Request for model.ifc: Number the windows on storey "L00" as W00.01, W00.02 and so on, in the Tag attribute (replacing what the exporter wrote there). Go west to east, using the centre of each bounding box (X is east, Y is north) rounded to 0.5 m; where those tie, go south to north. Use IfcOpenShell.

First a look at what the model holds.

```python
import ifcopenshell
import ifcopenshell.util.element
import ifcopenshell.util.placement

model = ifcopenshell.open("model.ifc")
print(model.schema)
storey = next(s for s in model.by_type("IfcBuildingStorey") if s.Name == "L00")
windows = [e for e in ifcopenshell.util.element.get_decomposition(storey) if e.is_a("IfcWindow")]
for e in sorted(windows, key=lambda e: e.id()):
    origin = ifcopenshell.util.placement.get_local_placement(e.ObjectPlacement)[:3, 3]
    print(e.id(), e.Tag, e.Name, origin.round(2) + 0.0, sep=" | ")
```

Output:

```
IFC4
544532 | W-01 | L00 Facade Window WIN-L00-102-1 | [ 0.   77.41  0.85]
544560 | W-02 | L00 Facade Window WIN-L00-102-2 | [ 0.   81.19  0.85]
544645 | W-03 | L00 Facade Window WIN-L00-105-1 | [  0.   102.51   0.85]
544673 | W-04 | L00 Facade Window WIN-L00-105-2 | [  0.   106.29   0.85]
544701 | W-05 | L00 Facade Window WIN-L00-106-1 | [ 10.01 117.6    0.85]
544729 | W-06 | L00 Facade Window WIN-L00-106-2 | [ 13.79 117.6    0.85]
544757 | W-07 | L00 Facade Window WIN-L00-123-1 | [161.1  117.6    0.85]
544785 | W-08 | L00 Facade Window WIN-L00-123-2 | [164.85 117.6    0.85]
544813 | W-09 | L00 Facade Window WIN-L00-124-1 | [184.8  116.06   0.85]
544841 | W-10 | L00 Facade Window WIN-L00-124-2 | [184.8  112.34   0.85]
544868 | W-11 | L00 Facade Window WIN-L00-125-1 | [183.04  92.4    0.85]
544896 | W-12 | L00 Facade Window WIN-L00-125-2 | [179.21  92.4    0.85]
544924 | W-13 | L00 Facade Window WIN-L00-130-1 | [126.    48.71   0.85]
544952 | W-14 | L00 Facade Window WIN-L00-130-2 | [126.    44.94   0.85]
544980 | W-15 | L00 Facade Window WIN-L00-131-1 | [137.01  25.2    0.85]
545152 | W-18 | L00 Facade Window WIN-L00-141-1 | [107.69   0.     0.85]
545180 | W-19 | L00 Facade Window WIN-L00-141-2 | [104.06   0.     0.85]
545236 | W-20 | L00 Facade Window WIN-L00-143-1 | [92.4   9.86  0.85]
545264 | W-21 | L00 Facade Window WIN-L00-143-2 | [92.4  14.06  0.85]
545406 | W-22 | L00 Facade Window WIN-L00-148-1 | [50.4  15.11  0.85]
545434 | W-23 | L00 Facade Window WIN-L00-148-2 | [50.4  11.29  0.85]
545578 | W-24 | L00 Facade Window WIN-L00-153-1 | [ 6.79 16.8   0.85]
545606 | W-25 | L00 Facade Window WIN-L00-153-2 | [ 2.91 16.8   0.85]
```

```python
import ifcopenshell
import ifcopenshell.geom
import ifcopenshell.util.element
import ifcopenshell.util.shape

model = ifcopenshell.open("model.ifc")
settings = ifcopenshell.geom.settings()
settings.set("use-world-coords", True)


def centre(element):
    shape = ifcopenshell.geom.create_shape(settings, element)
    return ifcopenshell.util.shape.get_bbox_centroid(shape.geometry)


storey = next(s for s in model.by_type("IfcBuildingStorey") if s.Name == "L00")
windows = [e for e in ifcopenshell.util.element.get_decomposition(storey) if e.is_a("IfcWindow")]

# Insertion points can sit at a corner or the storey origin, so sort by the geometry (in metres).
centres = {e: centre(e) for e in windows}
windows.sort(key=lambda e: (round(centres[e][0] / 0.5), centres[e][1]))

for i, e in enumerate(windows, start=1):
    number = f"W00.{i:02d}"
    e.Tag = number
    print(e.id(), number)

model.write("model_v2.ifc")
```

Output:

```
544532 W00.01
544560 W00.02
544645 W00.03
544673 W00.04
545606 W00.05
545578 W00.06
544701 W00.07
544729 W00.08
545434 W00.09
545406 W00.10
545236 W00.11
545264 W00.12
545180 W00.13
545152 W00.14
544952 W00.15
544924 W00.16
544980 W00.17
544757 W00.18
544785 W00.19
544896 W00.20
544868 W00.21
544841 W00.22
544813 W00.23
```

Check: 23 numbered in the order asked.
